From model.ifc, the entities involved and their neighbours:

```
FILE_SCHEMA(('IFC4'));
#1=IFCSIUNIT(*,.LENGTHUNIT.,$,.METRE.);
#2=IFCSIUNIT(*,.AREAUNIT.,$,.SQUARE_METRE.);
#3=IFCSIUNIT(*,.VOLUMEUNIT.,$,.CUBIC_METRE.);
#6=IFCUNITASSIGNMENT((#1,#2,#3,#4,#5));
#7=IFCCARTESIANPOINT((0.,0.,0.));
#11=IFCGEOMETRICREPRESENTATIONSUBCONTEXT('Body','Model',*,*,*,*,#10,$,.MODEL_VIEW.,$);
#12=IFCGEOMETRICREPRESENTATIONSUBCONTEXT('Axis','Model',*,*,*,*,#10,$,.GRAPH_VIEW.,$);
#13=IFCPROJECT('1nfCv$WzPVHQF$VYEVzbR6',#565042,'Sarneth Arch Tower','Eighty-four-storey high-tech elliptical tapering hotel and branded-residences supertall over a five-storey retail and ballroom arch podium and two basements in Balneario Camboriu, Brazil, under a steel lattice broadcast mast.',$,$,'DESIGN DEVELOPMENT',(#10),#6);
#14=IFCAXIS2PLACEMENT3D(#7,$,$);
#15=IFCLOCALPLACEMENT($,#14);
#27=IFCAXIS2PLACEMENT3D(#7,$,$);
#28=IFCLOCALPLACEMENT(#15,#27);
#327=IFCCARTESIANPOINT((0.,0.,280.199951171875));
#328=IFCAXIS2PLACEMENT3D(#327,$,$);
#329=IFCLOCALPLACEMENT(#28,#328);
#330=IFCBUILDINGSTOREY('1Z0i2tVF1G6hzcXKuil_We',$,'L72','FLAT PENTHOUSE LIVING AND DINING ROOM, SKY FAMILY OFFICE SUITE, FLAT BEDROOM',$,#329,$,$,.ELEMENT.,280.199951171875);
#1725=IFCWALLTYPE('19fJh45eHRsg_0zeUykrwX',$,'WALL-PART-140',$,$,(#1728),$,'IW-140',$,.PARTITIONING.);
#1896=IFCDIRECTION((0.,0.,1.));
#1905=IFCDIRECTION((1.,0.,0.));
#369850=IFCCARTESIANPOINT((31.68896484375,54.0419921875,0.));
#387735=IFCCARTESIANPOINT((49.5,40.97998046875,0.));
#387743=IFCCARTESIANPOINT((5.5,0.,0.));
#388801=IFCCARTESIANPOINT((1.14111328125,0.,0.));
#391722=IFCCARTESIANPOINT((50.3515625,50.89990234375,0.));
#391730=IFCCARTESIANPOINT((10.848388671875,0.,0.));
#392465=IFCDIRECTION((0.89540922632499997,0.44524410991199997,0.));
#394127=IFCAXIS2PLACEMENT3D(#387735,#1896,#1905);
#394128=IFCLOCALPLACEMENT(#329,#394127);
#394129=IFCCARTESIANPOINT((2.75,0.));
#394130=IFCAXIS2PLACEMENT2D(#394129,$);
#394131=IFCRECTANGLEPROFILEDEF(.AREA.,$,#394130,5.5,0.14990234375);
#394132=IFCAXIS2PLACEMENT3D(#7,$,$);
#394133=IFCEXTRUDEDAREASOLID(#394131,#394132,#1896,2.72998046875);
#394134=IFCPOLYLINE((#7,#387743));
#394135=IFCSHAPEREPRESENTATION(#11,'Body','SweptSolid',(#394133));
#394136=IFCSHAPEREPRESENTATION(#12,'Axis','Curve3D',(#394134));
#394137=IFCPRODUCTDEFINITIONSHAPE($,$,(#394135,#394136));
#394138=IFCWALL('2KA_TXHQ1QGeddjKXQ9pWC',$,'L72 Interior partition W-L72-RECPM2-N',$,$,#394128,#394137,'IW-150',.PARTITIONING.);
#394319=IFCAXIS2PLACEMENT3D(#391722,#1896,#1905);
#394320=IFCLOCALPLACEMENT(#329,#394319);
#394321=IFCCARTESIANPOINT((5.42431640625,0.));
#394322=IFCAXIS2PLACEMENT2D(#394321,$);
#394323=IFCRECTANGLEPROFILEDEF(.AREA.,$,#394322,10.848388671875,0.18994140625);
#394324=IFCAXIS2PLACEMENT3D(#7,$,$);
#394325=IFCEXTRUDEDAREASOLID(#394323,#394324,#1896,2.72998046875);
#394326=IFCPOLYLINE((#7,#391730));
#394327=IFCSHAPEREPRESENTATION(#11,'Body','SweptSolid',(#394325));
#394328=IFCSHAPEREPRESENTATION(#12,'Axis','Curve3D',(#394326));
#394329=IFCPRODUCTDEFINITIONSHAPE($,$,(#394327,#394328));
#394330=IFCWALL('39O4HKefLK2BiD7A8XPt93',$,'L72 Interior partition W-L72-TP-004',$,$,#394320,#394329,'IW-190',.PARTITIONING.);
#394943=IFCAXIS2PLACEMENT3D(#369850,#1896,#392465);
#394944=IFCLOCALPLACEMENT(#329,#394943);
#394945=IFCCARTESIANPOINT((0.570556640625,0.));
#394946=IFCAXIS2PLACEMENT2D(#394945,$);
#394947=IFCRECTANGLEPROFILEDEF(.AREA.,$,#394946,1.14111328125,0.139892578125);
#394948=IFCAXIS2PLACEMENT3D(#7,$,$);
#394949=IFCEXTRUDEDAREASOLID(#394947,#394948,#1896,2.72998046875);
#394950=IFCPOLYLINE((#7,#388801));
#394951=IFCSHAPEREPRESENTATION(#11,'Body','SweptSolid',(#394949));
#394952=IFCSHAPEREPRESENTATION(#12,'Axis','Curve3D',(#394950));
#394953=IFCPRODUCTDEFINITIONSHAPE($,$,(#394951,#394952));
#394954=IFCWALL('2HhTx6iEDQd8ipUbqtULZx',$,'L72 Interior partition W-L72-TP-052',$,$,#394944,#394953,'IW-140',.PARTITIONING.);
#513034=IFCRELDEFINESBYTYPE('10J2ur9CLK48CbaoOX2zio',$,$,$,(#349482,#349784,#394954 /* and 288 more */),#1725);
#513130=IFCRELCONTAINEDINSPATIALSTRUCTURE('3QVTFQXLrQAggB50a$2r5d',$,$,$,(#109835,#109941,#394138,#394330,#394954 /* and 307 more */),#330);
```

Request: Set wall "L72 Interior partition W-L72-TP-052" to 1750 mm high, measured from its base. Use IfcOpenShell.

```python
import ifcopenshell
import ifcopenshell.geom
import ifcopenshell.util.representation
import ifcopenshell.util.shape
import ifcopenshell.util.unit

model = ifcopenshell.open("model.ifc")
unit_scale = ifcopenshell.util.unit.calculate_unit_scale(model)
settings = ifcopenshell.geom.settings()


def volume(element):
    """Net volume in cubic metres, openings subtracted."""
    shape = ifcopenshell.geom.create_shape(settings, element)
    return ifcopenshell.util.shape.get_volume(shape.geometry)


wall = model.by_guid("2HhTx6iEDQd8ipUbqtULZx")
before = volume(wall)

body = ifcopenshell.util.representation.get_representation(wall, "Model", "Body")
solid = body.Items[0]
old_height = solid.Depth
solid.Depth = 1.75 / unit_scale
after = volume(wall)

print(f"height {old_height:g} -> {solid.Depth:g}, volume {before:.3f} -> {after:.3f} m3")

model.write("model_v2.ifc")
```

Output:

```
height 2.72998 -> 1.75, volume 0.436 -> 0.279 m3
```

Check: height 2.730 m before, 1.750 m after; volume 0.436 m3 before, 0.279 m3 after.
